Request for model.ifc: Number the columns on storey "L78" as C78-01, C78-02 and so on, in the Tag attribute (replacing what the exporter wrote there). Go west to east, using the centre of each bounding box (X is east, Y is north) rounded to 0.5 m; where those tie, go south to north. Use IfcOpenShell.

First a look at what the model holds.

```python
import ifcopenshell
import ifcopenshell.util.element
import ifcopenshell.util.placement

model = ifcopenshell.open("model.ifc")
print(model.schema)
storey = next(s for s in model.by_type("IfcBuildingStorey") if s.Name == "L78")
columns = [e for e in ifcopenshell.util.element.get_decomposition(storey) if e.is_a("IfcColumn")]
for e in sorted(columns, key=lambda e: e.id()):
    origin = ifcopenshell.util.placement.get_local_placement(e.ObjectPlacement)[:3, 3]
    print(e.id(), e.Tag, e.Name, origin.round(2) + 0.0, sep=" | ")
```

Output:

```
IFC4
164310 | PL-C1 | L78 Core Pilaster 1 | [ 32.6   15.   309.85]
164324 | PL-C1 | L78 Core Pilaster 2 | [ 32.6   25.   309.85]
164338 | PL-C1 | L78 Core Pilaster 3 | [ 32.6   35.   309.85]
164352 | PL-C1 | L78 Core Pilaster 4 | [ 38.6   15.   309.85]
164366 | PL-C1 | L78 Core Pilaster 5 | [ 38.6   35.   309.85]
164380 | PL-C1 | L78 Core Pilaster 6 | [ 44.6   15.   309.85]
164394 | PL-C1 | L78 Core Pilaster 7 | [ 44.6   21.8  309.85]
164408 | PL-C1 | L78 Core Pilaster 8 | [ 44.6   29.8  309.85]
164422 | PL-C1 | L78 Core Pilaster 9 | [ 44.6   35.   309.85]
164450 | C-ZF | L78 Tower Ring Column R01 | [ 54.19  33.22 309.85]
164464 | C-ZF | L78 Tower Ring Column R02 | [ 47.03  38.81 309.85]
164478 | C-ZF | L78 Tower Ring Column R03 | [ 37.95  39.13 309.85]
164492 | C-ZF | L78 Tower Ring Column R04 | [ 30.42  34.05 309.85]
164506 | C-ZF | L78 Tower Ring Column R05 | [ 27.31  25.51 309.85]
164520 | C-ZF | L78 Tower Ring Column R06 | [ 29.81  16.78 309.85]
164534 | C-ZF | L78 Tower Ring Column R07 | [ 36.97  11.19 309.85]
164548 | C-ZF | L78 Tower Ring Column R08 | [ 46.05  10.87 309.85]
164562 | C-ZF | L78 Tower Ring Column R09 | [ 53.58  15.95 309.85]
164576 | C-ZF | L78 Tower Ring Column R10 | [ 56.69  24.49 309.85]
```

```python
import ifcopenshell
import ifcopenshell.geom
import ifcopenshell.util.element
import ifcopenshell.util.shape

model = ifcopenshell.open("model.ifc")
settings = ifcopenshell.geom.settings()
settings.set("use-world-coords", True)


def centre(element):
    shape = ifcopenshell.geom.create_shape(settings, element)
    return ifcopenshell.util.shape.get_bbox_centroid(shape.geometry)


storey = next(s for s in model.by_type("IfcBuildingStorey") if s.Name == "L78")
columns = [e for e in ifcopenshell.util.element.get_decomposition(storey) if e.is_a("IfcColumn")]

# Insertion points can sit at a corner or the storey origin, so sort by the geometry (in metres).
centres = {e: centre(e) for e in columns}
columns.sort(key=lambda e: (round(centres[e][0] / 0.5), centres[e][1]))

for i, e in enumerate(columns, start=1):
    number = f"C78-{i:02d}"
    e.Tag = number
    print(e.id(), number)

model.write("model_updated.ifc")
```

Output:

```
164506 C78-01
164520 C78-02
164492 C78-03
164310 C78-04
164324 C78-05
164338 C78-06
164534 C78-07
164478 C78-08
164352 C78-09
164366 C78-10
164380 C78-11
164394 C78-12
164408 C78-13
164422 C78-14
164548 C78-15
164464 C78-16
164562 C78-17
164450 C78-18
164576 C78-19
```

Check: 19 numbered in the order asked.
